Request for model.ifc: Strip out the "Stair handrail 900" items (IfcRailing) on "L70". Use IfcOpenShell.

First a look at what the model holds.

```python
import ifcopenshell
import ifcopenshell.util.element

model = ifcopenshell.open("model.ifc")
print(model.schema)
storey = next(s for s in model.by_type("IfcBuildingStorey") if s.Name == "L70")
railings = [e for e in ifcopenshell.util.element.get_decomposition(storey) if e.is_a("IfcRailing")]
seen = {}
for e in railings:
    element_type = ifcopenshell.util.element.get_type(e)
    name = element_type.Name if element_type not in (None, e) else None
    seen[name] = seen.get(name, 0) + 1
for name, count in sorted(seen.items(), key=str):
    print(count, "x", name)
```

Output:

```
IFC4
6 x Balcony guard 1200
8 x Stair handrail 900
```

```python
import ifcopenshell
import ifcopenshell.api.root
import ifcopenshell.util.element

model = ifcopenshell.open("model.ifc")

storey = next(s for s in model.by_type("IfcBuildingStorey") if s.Name == "L70")
railings = [e for e in ifcopenshell.util.element.get_decomposition(storey) if e.is_a("IfcRailing")]
targets = [e for e in railings if (t := ifcopenshell.util.element.get_type(e)) not in (None, e) and t.Name == "Stair handrail 900"]

for e in targets:
    ifcopenshell.api.root.remove_product(model, product=e)
print(len(targets), "removed")

model.write("model_updated.ifc")
```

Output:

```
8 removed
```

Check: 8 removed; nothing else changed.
